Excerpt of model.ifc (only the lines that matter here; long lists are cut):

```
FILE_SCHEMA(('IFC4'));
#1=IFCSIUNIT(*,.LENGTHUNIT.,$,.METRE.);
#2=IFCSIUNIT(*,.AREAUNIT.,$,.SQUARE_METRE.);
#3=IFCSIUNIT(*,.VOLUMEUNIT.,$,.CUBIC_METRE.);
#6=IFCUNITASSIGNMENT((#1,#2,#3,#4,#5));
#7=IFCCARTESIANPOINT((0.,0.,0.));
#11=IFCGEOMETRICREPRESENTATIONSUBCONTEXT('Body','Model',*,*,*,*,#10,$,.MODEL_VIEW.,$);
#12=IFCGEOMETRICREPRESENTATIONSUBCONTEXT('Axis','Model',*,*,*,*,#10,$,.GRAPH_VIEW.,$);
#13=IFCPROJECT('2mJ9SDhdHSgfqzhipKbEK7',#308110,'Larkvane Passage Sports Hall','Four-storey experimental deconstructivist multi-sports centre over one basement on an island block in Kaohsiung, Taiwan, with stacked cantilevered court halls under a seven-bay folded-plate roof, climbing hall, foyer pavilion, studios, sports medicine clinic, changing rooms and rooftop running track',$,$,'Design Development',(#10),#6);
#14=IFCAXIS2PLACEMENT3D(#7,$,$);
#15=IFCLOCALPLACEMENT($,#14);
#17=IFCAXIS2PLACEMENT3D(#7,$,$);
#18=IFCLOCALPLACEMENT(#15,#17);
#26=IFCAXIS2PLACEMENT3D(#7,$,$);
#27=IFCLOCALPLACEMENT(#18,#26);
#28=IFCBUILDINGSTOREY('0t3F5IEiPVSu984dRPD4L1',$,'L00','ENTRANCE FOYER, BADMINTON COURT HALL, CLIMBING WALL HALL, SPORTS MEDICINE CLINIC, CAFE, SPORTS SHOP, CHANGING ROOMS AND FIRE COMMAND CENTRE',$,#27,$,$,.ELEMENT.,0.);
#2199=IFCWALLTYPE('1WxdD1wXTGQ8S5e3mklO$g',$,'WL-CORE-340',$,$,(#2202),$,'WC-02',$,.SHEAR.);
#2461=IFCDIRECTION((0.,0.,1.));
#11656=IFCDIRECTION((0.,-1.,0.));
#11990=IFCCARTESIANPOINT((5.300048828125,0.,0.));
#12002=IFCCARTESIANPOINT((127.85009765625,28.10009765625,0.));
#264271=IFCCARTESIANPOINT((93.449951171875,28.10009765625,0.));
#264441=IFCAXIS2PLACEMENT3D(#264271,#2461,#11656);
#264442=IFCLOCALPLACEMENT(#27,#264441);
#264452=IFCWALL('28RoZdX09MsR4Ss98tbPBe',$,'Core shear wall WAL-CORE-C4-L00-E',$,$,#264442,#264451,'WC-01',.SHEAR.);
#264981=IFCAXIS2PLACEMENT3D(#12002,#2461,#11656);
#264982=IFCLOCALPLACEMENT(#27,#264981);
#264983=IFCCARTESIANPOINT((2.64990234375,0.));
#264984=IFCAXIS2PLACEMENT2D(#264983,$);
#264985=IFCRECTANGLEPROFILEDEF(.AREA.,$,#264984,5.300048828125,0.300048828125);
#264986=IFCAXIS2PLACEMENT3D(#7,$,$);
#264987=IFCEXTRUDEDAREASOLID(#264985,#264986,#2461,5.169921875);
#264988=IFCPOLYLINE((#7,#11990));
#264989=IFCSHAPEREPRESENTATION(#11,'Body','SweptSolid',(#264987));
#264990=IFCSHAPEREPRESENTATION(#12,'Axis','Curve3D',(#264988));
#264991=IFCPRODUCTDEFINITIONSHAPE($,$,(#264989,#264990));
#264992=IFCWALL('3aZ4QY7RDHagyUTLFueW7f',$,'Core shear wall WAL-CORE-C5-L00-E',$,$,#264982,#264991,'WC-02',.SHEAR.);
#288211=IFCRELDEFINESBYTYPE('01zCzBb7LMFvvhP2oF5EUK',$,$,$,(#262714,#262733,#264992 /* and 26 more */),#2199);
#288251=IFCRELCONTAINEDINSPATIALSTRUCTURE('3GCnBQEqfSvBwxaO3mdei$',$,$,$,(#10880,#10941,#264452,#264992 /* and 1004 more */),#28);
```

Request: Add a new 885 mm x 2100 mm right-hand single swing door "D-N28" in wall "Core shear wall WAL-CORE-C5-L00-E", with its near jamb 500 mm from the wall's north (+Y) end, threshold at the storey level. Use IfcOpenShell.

```python
import numpy as np
import ifcopenshell
import ifcopenshell.api.feature
import ifcopenshell.api.geometry
import ifcopenshell.api.root
import ifcopenshell.api.spatial
import ifcopenshell.geom
import ifcopenshell.util.element
import ifcopenshell.util.placement
import ifcopenshell.util.representation
import ifcopenshell.util.shape
import ifcopenshell.util.unit

model = ifcopenshell.open("model.ifc")
unit_scale = ifcopenshell.util.unit.calculate_unit_scale(model)
settings = ifcopenshell.geom.settings()


def volume(element):
    """Net volume in cubic metres, openings subtracted."""
    shape = ifcopenshell.geom.create_shape(settings, element)
    return ifcopenshell.util.shape.get_volume(shape.geometry)


wall = model.by_guid("3aZ4QY7RDHagyUTLFueW7f")
storey = ifcopenshell.util.element.get_container(wall, ifc_class="IfcBuildingStorey")
context = ifcopenshell.util.representation.get_context(model, "Model", "Body", "MODEL_VIEW")
before = volume(wall)

width, height, from_end, sill = 0.885, 2.1, 0.5, 0.0  # metres

# The wall runs along its own X axis, and the end named is its -X end.
wall_shape = ifcopenshell.geom.create_shape(settings, wall)
x, y, z = ifcopenshell.util.shape.get_vertices(wall_shape.geometry).T
start = x.min() + from_end
face, thickness = float(y.min()), float(y.max() - y.min())
wall_matrix = ifcopenshell.util.placement.get_local_placement(wall.ObjectPlacement)
level = ifcopenshell.util.placement.get_local_placement(storey.ObjectPlacement)[2, 3]


def in_wall(x, y):
    """Placement at x, y metres in the wall's axes, at sill height."""
    matrix = wall_matrix.copy()
    matrix[:, 3] = wall_matrix @ np.array([x / unit_scale, y / unit_scale, 0.0, 1.0])
    matrix[2, 3] = level + sill / unit_scale
    return matrix


# Opening: a box that overshoots both wall faces by 50 mm.
opening = ifcopenshell.api.root.create_entity(model, ifc_class="IfcOpeningElement", predefined_type="OPENING")
box = ifcopenshell.api.geometry.add_wall_representation(
    model, context=context, length=width, height=height, thickness=thickness + 0.1
)
ifcopenshell.api.geometry.assign_representation(model, product=opening, representation=box)
ifcopenshell.api.geometry.edit_object_placement(model, product=opening, matrix=in_wall(start, face - 0.05), is_si=False)
ifcopenshell.api.feature.add_feature(model, feature=opening, element=wall)

door = ifcopenshell.api.root.create_entity(model, ifc_class="IfcDoor", name="D-N28", predefined_type="DOOR")
door.OverallWidth, door.OverallHeight = width / unit_scale, height / unit_scale
door.OperationType = "SINGLE_SWING_RIGHT"
body = ifcopenshell.api.geometry.add_door_representation(
    model,
    context=context,
    overall_width=door.OverallWidth,
    overall_height=door.OverallHeight,
    operation_type="SINGLE_SWING_RIGHT",
    lining_properties={"LiningDepth": thickness / unit_scale, "ThresholdDepth": thickness / unit_scale},
)
ifcopenshell.api.geometry.assign_representation(model, product=door, representation=body)
ifcopenshell.api.spatial.assign_container(model, products=[door], relating_structure=storey)
ifcopenshell.api.feature.add_filling(model, opening=opening, element=door)

# The lining spans the wall, so the door starts at the wall face.
ifcopenshell.api.geometry.edit_object_placement(model, product=door, matrix=in_wall(start, face), is_si=False)

after = volume(wall)

print(f"wall volume {before:.3f} -> {after:.3f} m3")

model.write("model_edited.ifc")
```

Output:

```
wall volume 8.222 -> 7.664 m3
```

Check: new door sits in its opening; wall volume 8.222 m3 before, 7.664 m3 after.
